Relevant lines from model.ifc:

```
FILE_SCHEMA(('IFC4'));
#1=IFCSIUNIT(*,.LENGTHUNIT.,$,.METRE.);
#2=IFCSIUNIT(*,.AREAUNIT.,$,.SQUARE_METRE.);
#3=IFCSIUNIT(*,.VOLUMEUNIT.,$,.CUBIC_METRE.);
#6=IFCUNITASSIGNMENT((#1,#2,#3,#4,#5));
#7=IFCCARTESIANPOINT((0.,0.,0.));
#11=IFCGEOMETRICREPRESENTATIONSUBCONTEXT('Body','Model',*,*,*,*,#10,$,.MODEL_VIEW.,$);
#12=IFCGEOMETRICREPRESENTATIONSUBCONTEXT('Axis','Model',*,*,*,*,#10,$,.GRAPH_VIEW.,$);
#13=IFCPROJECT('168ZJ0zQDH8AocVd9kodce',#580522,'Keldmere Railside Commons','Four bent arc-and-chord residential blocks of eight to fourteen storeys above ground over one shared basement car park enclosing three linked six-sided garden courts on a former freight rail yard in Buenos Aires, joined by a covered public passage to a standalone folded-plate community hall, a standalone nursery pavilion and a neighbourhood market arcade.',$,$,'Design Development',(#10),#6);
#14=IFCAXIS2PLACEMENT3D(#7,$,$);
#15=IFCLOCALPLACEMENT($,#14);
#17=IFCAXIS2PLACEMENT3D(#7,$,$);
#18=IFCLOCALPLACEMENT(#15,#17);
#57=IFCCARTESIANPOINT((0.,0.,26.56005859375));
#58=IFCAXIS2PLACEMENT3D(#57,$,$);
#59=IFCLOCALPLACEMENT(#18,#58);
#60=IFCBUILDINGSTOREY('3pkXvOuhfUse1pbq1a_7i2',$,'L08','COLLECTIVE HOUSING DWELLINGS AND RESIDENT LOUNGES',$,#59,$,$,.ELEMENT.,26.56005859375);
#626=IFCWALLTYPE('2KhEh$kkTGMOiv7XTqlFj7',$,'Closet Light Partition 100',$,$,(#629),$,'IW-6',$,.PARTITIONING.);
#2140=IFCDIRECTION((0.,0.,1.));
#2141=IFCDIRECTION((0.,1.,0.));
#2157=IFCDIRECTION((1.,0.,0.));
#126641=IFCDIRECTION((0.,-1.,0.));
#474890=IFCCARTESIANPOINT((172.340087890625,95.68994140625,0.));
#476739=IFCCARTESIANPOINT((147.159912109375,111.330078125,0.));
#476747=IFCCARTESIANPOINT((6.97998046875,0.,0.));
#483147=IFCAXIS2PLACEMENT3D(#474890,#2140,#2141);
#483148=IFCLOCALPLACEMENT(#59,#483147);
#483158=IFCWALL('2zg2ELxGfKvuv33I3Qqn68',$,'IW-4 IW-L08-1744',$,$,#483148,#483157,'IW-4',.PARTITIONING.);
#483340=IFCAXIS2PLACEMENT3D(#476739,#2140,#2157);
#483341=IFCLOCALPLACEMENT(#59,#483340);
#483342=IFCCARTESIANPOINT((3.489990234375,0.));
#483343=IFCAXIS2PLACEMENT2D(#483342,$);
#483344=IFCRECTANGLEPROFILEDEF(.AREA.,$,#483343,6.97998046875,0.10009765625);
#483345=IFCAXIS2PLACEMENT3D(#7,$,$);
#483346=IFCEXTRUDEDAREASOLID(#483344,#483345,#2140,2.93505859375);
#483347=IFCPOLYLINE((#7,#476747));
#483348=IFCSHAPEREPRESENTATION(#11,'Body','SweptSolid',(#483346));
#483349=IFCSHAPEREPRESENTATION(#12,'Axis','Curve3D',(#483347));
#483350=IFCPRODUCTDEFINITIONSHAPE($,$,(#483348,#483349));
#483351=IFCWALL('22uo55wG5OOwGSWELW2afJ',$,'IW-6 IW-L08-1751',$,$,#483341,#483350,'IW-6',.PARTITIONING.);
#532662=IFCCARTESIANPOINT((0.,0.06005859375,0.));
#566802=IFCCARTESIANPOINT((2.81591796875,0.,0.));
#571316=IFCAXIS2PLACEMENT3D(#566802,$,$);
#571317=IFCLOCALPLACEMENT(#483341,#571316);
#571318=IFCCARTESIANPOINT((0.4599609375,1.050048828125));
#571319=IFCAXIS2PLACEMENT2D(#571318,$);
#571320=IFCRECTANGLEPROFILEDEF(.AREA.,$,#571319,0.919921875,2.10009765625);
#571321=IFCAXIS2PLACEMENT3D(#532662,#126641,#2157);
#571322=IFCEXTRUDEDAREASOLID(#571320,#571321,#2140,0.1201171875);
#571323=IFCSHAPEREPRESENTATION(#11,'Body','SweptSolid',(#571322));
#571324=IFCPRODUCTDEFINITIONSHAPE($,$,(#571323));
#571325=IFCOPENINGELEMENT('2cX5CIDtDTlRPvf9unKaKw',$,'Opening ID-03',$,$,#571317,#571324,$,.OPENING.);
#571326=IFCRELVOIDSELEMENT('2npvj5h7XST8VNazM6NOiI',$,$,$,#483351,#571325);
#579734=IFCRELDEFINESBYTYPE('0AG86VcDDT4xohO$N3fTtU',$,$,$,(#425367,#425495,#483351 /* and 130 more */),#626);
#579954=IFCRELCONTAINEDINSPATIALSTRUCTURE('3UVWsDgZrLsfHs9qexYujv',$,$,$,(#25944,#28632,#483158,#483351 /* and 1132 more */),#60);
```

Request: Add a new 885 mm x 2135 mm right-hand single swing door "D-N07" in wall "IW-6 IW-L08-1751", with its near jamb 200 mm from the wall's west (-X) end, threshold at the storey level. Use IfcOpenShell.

```python
import numpy as np
import ifcopenshell
import ifcopenshell.api.feature
import ifcopenshell.api.geometry
import ifcopenshell.api.root
import ifcopenshell.api.spatial
import ifcopenshell.geom
import ifcopenshell.util.element
import ifcopenshell.util.placement
import ifcopenshell.util.representation
import ifcopenshell.util.shape
import ifcopenshell.util.unit

model = ifcopenshell.open("model.ifc")
unit_scale = ifcopenshell.util.unit.calculate_unit_scale(model)
settings = ifcopenshell.geom.settings()


def volume(element):
    """Net volume in cubic metres, openings subtracted."""
    shape = ifcopenshell.geom.create_shape(settings, element)
    return ifcopenshell.util.shape.get_volume(shape.geometry)


wall = model.by_guid("22uo55wG5OOwGSWELW2afJ")
storey = ifcopenshell.util.element.get_container(wall, ifc_class="IfcBuildingStorey")
context = ifcopenshell.util.representation.get_context(model, "Model", "Body", "MODEL_VIEW")
before = volume(wall)

width, height, from_end, sill = 0.885, 2.135, 0.2, 0.0  # metres

# The wall runs along its own X axis, and the end named is its -X end.
wall_shape = ifcopenshell.geom.create_shape(settings, wall)
x, y, z = ifcopenshell.util.shape.get_vertices(wall_shape.geometry).T
start = x.min() + from_end
face, thickness = float(y.min()), float(y.max() - y.min())
wall_matrix = ifcopenshell.util.placement.get_local_placement(wall.ObjectPlacement)
level = ifcopenshell.util.placement.get_local_placement(storey.ObjectPlacement)[2, 3]


def in_wall(x, y):
    """Placement at x, y metres in the wall's axes, at sill height."""
    matrix = wall_matrix.copy()
    matrix[:, 3] = wall_matrix @ np.array([x / unit_scale, y / unit_scale, 0.0, 1.0])
    matrix[2, 3] = level + sill / unit_scale
    return matrix


# Opening: a box that overshoots both wall faces by 50 mm.
opening = ifcopenshell.api.root.create_entity(model, ifc_class="IfcOpeningElement", predefined_type="OPENING")
box = ifcopenshell.api.geometry.add_wall_representation(
    model, context=context, length=width, height=height, thickness=thickness + 0.1
)
ifcopenshell.api.geometry.assign_representation(model, product=opening, representation=box)
ifcopenshell.api.geometry.edit_object_placement(model, product=opening, matrix=in_wall(start, face - 0.05), is_si=False)
ifcopenshell.api.feature.add_feature(model, feature=opening, element=wall)

door = ifcopenshell.api.root.create_entity(model, ifc_class="IfcDoor", name="D-N07", predefined_type="DOOR")
door.OverallWidth, door.OverallHeight = width / unit_scale, height / unit_scale
door.OperationType = "SINGLE_SWING_RIGHT"
body = ifcopenshell.api.geometry.add_door_representation(
    model,
    context=context,
    overall_width=door.OverallWidth,
    overall_height=door.OverallHeight,
    operation_type="SINGLE_SWING_RIGHT",
    lining_properties={"LiningDepth": thickness / unit_scale, "ThresholdDepth": thickness / unit_scale},
)
ifcopenshell.api.geometry.assign_representation(model, product=door, representation=body)
ifcopenshell.api.spatial.assign_container(model, products=[door], relating_structure=storey)
ifcopenshell.api.feature.add_filling(model, opening=opening, element=door)

# The lining spans the wall, so the door starts at the wall face.
ifcopenshell.api.geometry.edit_object_placement(model, product=door, matrix=in_wall(start, face), is_si=False)

after = volume(wall)

print(f"wall volume {before:.3f} -> {after:.3f} m3")

model.write("model-out.ifc")
```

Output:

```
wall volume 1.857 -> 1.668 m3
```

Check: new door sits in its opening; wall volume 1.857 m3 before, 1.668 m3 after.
